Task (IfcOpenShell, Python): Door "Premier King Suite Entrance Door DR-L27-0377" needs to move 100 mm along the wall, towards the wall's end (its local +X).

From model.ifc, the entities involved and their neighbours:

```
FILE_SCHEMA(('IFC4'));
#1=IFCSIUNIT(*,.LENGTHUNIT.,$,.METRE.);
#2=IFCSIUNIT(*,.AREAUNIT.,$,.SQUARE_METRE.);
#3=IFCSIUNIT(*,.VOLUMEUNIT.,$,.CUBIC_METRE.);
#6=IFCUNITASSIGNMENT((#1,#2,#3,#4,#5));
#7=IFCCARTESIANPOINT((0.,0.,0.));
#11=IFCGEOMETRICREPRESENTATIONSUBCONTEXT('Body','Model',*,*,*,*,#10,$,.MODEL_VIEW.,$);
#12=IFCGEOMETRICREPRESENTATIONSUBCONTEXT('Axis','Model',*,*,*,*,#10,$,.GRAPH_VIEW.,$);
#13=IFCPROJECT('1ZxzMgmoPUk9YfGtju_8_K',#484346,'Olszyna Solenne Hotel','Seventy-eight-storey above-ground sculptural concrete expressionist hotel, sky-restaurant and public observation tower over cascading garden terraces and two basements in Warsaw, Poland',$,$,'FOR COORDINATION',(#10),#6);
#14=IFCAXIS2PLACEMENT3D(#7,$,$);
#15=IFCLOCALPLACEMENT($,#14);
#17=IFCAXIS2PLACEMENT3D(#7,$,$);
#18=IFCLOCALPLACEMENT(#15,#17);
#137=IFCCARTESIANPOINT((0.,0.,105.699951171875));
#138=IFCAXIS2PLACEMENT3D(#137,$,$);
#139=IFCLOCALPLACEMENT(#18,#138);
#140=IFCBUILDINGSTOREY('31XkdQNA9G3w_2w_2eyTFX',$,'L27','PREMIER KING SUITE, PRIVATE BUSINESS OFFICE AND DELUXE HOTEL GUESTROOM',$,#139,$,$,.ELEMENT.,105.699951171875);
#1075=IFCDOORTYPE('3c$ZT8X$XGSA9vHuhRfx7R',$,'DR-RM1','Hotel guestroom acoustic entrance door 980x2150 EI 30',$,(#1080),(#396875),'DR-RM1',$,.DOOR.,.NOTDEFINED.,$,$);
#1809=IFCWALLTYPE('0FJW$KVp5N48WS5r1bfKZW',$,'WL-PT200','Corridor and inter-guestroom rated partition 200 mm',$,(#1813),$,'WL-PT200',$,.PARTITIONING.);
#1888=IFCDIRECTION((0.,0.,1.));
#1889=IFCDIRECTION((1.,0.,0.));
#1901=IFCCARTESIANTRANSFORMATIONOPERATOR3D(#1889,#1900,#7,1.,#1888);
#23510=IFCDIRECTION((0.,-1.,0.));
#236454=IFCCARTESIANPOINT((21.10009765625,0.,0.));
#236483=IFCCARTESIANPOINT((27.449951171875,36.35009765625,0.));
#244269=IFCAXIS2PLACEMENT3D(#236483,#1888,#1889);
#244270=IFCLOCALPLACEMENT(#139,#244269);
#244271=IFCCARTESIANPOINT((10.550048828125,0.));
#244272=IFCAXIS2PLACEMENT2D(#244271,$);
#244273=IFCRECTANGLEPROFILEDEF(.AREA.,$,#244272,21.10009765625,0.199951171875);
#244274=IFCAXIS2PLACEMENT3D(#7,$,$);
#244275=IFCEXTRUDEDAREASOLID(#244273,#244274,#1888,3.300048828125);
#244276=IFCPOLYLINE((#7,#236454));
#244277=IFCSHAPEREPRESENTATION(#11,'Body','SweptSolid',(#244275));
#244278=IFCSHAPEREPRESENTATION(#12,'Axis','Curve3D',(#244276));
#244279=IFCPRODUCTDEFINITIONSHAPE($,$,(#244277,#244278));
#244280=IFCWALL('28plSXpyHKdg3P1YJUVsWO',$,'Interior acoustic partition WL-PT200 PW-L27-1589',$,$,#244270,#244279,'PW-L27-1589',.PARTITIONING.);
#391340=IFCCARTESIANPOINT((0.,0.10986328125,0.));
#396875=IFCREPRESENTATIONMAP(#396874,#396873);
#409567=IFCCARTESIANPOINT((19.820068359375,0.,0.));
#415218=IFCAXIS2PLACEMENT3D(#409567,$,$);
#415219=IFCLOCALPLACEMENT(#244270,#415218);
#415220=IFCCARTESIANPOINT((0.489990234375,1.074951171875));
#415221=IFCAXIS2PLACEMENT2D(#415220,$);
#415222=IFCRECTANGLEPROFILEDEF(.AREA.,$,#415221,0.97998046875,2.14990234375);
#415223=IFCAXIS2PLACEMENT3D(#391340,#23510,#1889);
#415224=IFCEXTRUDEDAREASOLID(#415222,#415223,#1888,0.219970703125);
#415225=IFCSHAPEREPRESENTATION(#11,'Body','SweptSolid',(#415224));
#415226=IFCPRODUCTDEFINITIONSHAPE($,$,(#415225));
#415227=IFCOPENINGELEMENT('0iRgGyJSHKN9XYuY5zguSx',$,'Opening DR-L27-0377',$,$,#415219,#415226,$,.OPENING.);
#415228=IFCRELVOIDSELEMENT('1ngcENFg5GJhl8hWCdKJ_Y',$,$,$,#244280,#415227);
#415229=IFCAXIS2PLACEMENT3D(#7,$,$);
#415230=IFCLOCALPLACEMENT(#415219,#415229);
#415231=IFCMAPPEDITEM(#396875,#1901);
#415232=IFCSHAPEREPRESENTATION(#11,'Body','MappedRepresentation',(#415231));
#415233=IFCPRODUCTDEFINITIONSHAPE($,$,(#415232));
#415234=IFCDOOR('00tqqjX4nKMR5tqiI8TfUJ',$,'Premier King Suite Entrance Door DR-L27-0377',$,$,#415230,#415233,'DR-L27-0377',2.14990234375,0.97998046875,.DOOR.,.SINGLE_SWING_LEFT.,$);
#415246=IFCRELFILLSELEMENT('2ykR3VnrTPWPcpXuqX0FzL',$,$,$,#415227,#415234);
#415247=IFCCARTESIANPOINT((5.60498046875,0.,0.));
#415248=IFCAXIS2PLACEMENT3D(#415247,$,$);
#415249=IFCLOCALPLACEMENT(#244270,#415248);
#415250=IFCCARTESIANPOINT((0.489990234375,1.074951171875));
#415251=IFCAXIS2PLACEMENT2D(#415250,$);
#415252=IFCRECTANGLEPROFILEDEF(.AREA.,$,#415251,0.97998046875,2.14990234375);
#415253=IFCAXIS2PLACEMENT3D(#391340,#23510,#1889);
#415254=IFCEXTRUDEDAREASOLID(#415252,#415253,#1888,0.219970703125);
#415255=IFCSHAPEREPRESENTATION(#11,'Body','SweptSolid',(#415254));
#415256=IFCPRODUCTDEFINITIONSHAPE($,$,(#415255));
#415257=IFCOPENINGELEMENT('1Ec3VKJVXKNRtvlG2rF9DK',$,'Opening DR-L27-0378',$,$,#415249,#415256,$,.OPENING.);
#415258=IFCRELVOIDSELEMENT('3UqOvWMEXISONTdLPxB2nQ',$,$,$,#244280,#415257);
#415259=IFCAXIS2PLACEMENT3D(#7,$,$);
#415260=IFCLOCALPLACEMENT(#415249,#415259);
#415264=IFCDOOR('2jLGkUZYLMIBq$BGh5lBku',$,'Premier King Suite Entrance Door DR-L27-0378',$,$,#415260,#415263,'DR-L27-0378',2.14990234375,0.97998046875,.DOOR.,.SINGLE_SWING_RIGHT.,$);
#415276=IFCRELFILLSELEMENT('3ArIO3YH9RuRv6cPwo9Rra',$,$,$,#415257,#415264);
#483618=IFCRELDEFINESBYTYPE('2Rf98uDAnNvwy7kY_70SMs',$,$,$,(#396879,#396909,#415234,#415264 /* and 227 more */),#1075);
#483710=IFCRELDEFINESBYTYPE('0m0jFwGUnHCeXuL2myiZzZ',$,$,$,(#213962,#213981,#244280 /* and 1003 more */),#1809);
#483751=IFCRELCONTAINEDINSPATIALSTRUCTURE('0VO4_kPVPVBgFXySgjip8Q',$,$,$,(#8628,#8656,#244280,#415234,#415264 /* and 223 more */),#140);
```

```python
import ifcopenshell
import ifcopenshell.api.geometry
import ifcopenshell.util.placement
import ifcopenshell.util.unit

model = ifcopenshell.open("model.ifc")
unit_scale = ifcopenshell.util.unit.calculate_unit_scale(model)

door = model.by_guid("00tqqjX4nKMR5tqiI8TfUJ")
opening = door.FillsVoids[0].RelatingOpeningElement
wall = opening.VoidsElements[0].RelatingBuildingElement

wall_matrix = ifcopenshell.util.placement.get_local_placement(wall.ObjectPlacement)
shift = wall_matrix[:3, 0] * 0.1 / unit_scale
before = ifcopenshell.util.placement.get_local_placement(door.ObjectPlacement)[:3, 3].copy()

# The door is placed relative to its opening, so it follows when the opening moves.
matrix = ifcopenshell.util.placement.get_local_placement(opening.ObjectPlacement)
matrix[:3, 3] += shift
ifcopenshell.api.geometry.edit_object_placement(
    model, product=opening, matrix=matrix, is_si=False, should_transform_children=True
)

after = ifcopenshell.util.placement.get_local_placement(door.ObjectPlacement)[:3, 3]
print("door moved by", (after - before).round(3) + 0.0)

model.write("model_rev.ifc")
```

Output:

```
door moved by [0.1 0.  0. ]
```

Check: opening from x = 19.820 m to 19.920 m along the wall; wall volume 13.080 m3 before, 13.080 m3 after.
